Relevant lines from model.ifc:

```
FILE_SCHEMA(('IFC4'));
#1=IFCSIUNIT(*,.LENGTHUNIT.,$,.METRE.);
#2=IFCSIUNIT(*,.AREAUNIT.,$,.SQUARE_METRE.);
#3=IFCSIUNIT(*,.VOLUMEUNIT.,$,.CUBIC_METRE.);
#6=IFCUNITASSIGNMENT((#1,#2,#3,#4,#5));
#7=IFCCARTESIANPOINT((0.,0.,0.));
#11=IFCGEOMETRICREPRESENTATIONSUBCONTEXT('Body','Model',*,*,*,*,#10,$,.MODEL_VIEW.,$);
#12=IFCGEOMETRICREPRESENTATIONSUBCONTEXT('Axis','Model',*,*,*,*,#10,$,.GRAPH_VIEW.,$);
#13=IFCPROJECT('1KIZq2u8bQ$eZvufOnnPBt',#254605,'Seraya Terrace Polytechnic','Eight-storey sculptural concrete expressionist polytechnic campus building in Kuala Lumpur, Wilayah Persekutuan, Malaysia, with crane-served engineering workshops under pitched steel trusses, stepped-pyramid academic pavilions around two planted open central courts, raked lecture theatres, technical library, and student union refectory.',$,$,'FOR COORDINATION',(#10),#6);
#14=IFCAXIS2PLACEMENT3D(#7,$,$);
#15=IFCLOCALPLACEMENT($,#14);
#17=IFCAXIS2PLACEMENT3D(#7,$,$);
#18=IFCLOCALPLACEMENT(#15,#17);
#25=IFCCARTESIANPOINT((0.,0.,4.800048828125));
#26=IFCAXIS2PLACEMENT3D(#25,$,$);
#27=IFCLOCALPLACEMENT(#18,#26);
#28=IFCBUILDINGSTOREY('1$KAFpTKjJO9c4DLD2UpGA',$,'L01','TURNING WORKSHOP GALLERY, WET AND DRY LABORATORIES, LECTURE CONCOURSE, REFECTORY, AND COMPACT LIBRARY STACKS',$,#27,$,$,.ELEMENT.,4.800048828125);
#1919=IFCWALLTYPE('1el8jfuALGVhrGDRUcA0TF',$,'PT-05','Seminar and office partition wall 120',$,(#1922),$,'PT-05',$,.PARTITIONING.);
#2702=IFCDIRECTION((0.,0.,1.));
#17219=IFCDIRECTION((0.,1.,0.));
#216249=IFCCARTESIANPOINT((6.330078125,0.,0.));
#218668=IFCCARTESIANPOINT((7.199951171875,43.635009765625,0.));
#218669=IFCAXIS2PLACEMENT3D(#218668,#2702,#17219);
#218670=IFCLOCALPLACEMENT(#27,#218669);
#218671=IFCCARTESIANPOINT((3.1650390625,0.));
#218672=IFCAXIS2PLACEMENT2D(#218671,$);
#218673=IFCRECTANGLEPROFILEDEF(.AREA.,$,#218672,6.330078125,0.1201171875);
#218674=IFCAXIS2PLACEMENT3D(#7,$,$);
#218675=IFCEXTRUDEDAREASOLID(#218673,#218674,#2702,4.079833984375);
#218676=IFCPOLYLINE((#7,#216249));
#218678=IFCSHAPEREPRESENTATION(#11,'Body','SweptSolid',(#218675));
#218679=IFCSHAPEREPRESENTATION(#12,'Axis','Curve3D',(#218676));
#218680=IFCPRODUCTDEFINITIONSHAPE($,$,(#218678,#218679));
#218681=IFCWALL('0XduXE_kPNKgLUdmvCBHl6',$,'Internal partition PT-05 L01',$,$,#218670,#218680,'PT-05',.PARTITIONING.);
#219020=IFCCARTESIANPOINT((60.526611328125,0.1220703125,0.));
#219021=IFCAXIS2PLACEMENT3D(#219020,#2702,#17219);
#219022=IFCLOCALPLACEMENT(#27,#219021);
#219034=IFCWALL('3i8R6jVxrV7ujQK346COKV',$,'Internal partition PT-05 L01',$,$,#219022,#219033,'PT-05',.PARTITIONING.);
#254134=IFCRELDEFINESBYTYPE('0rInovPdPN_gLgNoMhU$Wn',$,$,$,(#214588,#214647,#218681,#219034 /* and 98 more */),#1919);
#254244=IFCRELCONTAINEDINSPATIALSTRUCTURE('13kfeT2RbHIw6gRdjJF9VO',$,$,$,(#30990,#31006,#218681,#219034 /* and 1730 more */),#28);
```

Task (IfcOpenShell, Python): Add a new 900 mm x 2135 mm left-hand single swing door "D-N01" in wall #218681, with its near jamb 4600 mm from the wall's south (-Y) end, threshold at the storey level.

```python
import numpy as np
import ifcopenshell
import ifcopenshell.api.feature
import ifcopenshell.api.geometry
import ifcopenshell.api.root
import ifcopenshell.api.spatial
import ifcopenshell.geom
import ifcopenshell.util.element
import ifcopenshell.util.placement
import ifcopenshell.util.representation
import ifcopenshell.util.shape
import ifcopenshell.util.unit

model = ifcopenshell.open("model.ifc")
unit_scale = ifcopenshell.util.unit.calculate_unit_scale(model)
settings = ifcopenshell.geom.settings()


def volume(element):
    """Net volume in cubic metres, openings subtracted."""
    shape = ifcopenshell.geom.create_shape(settings, element)
    return ifcopenshell.util.shape.get_volume(shape.geometry)


wall = model.by_guid("0XduXE_kPNKgLUdmvCBHl6")
storey = ifcopenshell.util.element.get_container(wall, ifc_class="IfcBuildingStorey")
context = ifcopenshell.util.representation.get_context(model, "Model", "Body", "MODEL_VIEW")
before = volume(wall)

width, height, from_end, sill = 0.9, 2.135, 4.6, 0.0  # metres

# The wall runs along its own X axis, and the end named is its -X end.
wall_shape = ifcopenshell.geom.create_shape(settings, wall)
x, y, z = ifcopenshell.util.shape.get_vertices(wall_shape.geometry).T
start = x.min() + from_end
face, thickness = float(y.min()), float(y.max() - y.min())
wall_matrix = ifcopenshell.util.placement.get_local_placement(wall.ObjectPlacement)
level = ifcopenshell.util.placement.get_local_placement(storey.ObjectPlacement)[2, 3]


def in_wall(x, y):
    """Placement at x, y metres in the wall's axes, at sill height."""
    matrix = wall_matrix.copy()
    matrix[:, 3] = wall_matrix @ np.array([x / unit_scale, y / unit_scale, 0.0, 1.0])
    matrix[2, 3] = level + sill / unit_scale
    return matrix


# Opening: a box that overshoots both wall faces by 50 mm.
opening = ifcopenshell.api.root.create_entity(model, ifc_class="IfcOpeningElement", predefined_type="OPENING")
box = ifcopenshell.api.geometry.add_wall_representation(
    model, context=context, length=width, height=height, thickness=thickness + 0.1
)
ifcopenshell.api.geometry.assign_representation(model, product=opening, representation=box)
ifcopenshell.api.geometry.edit_object_placement(model, product=opening, matrix=in_wall(start, face - 0.05), is_si=False)
ifcopenshell.api.feature.add_feature(model, feature=opening, element=wall)

door = ifcopenshell.api.root.create_entity(model, ifc_class="IfcDoor", name="D-N01", predefined_type="DOOR")
door.OverallWidth, door.OverallHeight = width / unit_scale, height / unit_scale
door.OperationType = "SINGLE_SWING_LEFT"
body = ifcopenshell.api.geometry.add_door_representation(
    model,
    context=context,
    overall_width=door.OverallWidth,
    overall_height=door.OverallHeight,
    operation_type="SINGLE_SWING_LEFT",
    lining_properties={"LiningDepth": thickness / unit_scale, "ThresholdDepth": thickness / unit_scale},
)
ifcopenshell.api.geometry.assign_representation(model, product=door, representation=body)
ifcopenshell.api.spatial.assign_container(model, products=[door], relating_structure=storey)
ifcopenshell.api.feature.add_filling(model, opening=opening, element=door)

# The lining spans the wall, so the door starts at the wall face.
ifcopenshell.api.geometry.edit_object_placement(model, product=door, matrix=in_wall(start, face), is_si=False)

after = volume(wall)

print(f"wall volume {before:.3f} -> {after:.3f} m3")

model.write("model-out.ifc")
```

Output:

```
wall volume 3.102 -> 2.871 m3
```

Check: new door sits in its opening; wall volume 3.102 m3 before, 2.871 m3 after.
